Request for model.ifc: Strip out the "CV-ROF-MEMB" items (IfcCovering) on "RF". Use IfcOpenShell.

First a look at what the model holds.

```python
import ifcopenshell
import ifcopenshell.util.element

model = ifcopenshell.open("model.ifc")
print(model.schema)
storey = next(s for s in model.by_type("IfcBuildingStorey") if s.Name == "RF")
coverings = [e for e in ifcopenshell.util.element.get_decomposition(storey) if e.is_a("IfcCovering")]
seen = {}
for e in coverings:
    element_type = ifcopenshell.util.element.get_type(e)
    name = element_type.Name if element_type not in (None, e) else None
    seen[name] = seen.get(name, 0) + 1
for name, count in sorted(seen.items(), key=str):
    print(count, "x", name)
```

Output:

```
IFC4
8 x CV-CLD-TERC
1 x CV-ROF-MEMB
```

```python
import ifcopenshell
import ifcopenshell.api.root
import ifcopenshell.util.element

model = ifcopenshell.open("model.ifc")

storey = next(s for s in model.by_type("IfcBuildingStorey") if s.Name == "RF")
coverings = [e for e in ifcopenshell.util.element.get_decomposition(storey) if e.is_a("IfcCovering")]
targets = [e for e in coverings if (t := ifcopenshell.util.element.get_type(e)) not in (None, e) and t.Name == "CV-ROF-MEMB"]

for e in targets:
    ifcopenshell.api.root.remove_product(model, product=e)
print(len(targets), "removed")

model.write("model-out.ifc")
```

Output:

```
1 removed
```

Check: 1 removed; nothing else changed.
